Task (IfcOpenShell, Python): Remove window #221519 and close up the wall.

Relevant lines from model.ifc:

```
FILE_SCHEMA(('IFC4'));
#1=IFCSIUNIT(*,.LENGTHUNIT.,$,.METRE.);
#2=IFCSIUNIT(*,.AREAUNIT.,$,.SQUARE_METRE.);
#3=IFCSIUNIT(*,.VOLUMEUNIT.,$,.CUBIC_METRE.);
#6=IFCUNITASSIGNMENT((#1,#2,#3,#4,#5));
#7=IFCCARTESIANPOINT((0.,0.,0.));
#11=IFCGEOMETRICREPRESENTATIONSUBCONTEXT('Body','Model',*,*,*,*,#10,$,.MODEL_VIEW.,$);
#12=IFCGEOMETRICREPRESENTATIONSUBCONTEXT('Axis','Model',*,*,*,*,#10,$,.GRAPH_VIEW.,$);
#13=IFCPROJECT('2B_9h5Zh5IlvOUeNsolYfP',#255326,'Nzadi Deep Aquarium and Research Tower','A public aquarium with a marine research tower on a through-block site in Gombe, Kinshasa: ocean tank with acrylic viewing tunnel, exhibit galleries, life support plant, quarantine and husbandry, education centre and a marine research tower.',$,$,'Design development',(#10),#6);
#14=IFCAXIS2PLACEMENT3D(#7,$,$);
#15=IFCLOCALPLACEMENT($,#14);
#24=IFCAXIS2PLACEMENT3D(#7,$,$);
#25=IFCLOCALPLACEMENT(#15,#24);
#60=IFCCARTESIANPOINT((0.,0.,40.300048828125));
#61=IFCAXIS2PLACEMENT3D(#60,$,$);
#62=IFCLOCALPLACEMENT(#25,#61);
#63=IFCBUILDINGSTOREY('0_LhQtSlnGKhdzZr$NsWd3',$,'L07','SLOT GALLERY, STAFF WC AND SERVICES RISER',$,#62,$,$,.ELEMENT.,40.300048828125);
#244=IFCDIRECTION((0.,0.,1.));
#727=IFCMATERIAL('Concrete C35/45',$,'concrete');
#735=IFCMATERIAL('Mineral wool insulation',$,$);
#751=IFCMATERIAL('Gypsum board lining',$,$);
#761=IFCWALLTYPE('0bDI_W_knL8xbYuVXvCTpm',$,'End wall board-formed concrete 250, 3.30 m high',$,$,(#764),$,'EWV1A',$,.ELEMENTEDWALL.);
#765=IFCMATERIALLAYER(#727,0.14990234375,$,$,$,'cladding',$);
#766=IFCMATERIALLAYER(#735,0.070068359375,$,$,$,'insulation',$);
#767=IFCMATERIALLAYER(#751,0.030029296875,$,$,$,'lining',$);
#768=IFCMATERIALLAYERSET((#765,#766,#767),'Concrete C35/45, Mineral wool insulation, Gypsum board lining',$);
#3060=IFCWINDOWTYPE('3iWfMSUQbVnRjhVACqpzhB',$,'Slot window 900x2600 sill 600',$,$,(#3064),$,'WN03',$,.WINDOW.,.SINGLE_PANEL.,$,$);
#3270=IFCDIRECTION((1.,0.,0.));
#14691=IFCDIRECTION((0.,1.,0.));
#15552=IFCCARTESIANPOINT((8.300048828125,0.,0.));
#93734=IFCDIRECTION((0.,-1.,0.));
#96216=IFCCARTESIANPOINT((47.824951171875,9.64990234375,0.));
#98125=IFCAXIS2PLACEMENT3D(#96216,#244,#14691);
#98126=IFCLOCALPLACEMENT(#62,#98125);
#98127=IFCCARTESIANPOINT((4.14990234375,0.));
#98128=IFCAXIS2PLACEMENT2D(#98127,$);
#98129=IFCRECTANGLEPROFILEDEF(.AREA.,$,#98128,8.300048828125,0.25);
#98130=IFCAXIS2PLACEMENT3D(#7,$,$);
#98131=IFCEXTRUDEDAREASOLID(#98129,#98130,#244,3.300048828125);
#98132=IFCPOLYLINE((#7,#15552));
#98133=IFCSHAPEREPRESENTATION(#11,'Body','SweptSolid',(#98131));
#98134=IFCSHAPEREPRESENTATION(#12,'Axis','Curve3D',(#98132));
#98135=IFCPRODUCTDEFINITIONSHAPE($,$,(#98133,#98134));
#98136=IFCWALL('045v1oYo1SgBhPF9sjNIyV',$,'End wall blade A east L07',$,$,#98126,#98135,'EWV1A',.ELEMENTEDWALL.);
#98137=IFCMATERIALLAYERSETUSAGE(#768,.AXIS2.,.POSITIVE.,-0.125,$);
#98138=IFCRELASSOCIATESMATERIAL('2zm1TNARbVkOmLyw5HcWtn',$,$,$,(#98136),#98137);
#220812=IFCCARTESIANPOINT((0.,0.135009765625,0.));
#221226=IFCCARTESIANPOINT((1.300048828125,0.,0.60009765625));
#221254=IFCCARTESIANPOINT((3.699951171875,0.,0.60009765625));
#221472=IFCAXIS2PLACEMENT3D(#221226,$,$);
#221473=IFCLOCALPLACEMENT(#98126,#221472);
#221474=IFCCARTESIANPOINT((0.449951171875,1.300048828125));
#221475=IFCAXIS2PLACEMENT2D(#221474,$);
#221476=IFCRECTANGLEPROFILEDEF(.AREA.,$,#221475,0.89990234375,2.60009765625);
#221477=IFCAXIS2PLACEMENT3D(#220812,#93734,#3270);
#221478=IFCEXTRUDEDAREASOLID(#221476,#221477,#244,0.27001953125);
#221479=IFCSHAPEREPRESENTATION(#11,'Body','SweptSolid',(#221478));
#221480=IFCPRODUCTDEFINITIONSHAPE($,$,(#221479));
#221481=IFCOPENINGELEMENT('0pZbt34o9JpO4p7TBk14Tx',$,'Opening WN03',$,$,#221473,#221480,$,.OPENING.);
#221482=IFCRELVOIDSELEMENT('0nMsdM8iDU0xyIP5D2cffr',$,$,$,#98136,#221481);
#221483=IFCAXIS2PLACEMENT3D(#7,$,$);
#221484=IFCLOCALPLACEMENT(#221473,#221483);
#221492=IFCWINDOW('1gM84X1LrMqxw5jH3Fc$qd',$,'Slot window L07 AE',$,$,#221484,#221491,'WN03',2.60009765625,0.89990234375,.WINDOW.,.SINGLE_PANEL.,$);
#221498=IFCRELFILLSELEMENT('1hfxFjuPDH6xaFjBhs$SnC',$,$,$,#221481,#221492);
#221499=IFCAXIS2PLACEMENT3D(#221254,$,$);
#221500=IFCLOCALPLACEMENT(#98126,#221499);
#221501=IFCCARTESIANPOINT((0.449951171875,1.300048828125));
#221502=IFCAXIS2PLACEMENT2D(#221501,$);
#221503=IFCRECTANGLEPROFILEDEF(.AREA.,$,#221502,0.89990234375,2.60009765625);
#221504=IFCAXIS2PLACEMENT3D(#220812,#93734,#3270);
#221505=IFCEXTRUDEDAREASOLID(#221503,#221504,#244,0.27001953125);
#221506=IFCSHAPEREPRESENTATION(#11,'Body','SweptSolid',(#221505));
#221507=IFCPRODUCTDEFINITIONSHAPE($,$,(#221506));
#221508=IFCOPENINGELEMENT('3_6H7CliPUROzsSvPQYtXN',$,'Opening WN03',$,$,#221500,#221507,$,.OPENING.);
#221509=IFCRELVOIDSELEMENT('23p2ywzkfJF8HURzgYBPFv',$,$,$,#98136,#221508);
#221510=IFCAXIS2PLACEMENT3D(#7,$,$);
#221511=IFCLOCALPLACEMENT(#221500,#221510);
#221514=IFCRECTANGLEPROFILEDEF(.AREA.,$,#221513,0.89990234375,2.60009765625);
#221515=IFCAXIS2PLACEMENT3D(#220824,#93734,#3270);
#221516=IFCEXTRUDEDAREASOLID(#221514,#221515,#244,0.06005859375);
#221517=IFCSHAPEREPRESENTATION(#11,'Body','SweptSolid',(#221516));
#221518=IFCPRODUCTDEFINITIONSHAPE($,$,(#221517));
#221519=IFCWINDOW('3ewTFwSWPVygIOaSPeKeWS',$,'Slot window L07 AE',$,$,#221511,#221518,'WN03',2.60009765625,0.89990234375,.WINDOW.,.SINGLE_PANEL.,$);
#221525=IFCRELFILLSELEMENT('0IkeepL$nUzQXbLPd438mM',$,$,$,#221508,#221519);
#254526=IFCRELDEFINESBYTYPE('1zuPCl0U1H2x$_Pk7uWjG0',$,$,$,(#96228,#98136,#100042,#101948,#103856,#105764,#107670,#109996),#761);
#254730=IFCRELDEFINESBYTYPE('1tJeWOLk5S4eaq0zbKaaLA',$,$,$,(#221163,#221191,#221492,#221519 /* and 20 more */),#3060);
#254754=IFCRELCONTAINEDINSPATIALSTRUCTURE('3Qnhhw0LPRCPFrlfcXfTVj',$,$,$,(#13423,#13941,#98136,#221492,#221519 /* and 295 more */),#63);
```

```python
import ifcopenshell
import ifcopenshell.api.feature
import ifcopenshell.api.root
import ifcopenshell.geom
import ifcopenshell.util.shape

model = ifcopenshell.open("model.ifc")
settings = ifcopenshell.geom.settings()


def volume(element):
    """Net volume in cubic metres, openings subtracted."""
    shape = ifcopenshell.geom.create_shape(settings, element)
    return ifcopenshell.util.shape.get_volume(shape.geometry)


window = model.by_guid("3ewTFwSWPVygIOaSPeKeWS")
opening = window.FillsVoids[0].RelatingOpeningElement
wall = opening.VoidsElements[0].RelatingBuildingElement
before = volume(wall)

ifcopenshell.api.root.remove_product(model, product=window)
ifcopenshell.api.feature.remove_feature(model, feature=opening)

after = volume(wall)

print(f"wall volume {before:.3f} -> {after:.3f} m3")

model.write("model_v2.ifc")
```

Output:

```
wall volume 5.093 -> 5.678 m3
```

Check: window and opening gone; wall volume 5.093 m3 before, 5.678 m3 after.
